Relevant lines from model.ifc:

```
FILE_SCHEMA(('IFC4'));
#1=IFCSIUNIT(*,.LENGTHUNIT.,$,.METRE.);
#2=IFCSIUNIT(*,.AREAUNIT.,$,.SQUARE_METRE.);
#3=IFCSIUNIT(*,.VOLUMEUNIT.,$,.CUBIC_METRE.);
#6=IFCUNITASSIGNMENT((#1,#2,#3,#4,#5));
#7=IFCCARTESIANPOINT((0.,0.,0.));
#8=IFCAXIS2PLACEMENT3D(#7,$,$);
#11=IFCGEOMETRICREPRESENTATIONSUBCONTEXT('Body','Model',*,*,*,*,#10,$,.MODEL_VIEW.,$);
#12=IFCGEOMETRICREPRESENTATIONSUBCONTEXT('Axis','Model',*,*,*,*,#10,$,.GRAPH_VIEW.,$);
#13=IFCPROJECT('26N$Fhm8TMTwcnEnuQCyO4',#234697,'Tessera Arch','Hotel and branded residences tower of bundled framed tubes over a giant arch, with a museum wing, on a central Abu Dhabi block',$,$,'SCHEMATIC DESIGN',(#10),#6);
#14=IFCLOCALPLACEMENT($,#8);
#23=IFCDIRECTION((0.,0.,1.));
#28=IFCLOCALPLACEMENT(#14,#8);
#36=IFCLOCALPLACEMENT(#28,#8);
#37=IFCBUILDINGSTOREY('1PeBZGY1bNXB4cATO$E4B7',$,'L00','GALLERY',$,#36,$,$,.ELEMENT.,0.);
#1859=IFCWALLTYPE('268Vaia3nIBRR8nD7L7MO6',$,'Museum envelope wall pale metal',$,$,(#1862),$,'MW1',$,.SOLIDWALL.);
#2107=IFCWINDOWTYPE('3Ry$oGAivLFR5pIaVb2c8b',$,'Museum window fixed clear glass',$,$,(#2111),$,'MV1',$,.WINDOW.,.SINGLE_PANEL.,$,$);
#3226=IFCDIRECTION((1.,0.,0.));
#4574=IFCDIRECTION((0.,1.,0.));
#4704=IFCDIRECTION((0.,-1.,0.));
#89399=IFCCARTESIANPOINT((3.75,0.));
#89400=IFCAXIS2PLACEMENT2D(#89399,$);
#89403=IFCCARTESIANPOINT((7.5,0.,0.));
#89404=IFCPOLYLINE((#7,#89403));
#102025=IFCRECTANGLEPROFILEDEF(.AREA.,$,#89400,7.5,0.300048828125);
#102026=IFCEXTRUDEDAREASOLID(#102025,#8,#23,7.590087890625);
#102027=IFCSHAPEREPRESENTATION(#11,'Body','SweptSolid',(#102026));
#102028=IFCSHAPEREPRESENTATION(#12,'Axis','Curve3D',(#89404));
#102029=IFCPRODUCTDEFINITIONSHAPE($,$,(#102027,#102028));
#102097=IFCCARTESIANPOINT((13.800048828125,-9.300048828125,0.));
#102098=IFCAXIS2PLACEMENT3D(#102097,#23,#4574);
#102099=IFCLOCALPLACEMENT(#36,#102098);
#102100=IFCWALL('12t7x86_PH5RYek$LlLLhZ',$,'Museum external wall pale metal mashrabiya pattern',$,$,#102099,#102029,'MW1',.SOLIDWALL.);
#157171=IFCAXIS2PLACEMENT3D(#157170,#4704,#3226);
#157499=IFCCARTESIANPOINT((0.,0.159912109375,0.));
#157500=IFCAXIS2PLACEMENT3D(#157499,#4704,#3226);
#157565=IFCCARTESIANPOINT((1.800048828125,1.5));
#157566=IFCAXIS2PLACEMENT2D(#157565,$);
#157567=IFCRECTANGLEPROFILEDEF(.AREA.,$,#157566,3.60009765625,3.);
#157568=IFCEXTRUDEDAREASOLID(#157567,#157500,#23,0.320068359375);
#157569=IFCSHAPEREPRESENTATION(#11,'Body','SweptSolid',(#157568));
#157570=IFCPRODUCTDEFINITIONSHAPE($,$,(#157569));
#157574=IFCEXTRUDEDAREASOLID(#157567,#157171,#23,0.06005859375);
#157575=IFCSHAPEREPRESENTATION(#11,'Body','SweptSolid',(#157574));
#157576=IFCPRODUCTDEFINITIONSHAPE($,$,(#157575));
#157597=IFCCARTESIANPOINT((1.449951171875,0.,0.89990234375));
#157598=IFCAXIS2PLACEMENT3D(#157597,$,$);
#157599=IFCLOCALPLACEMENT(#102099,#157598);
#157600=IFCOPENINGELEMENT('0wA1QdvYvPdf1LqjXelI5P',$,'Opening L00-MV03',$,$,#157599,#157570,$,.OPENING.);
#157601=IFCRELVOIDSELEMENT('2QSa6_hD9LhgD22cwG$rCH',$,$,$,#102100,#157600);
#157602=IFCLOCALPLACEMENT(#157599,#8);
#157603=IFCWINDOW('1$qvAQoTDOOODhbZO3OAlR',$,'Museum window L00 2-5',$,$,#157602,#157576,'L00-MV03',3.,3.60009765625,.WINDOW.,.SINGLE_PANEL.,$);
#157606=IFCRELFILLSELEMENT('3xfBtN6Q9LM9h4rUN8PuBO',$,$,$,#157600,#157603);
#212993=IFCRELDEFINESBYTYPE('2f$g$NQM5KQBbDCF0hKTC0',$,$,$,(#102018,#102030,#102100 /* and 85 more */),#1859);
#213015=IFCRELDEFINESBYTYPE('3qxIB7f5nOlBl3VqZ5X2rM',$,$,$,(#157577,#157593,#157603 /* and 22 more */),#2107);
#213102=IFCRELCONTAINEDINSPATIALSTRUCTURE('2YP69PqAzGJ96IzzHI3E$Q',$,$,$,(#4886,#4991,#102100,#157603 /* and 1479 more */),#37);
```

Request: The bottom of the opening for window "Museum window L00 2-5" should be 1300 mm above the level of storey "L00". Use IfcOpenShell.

```python
import numpy as np
import ifcopenshell
import ifcopenshell.api.geometry
import ifcopenshell.geom
import ifcopenshell.util.element
import ifcopenshell.util.placement
import ifcopenshell.util.shape
import ifcopenshell.util.unit

model = ifcopenshell.open("model.ifc")
unit_scale = ifcopenshell.util.unit.calculate_unit_scale(model)

window = model.by_guid("1$qvAQoTDOOODhbZO3OAlR")
opening = window.FillsVoids[0].RelatingOpeningElement
storey = ifcopenshell.util.element.get_container(window, ifc_class="IfcBuildingStorey")
level = ifcopenshell.util.placement.get_local_placement(storey.ObjectPlacement)[2, 3]

# The opening's origin need not be at the sill, so measure its lowest point.
shape = ifcopenshell.geom.create_shape(ifcopenshell.geom.settings(), opening)
bottom = ifcopenshell.util.shape.get_shape_bottom_elevation(shape, shape.geometry) / unit_scale
dz = level + 1.3 - bottom

shift = np.array([0.0, 0.0, dz])
# The window is placed relative to its opening, so it follows when the opening moves.
matrix = ifcopenshell.util.placement.get_local_placement(opening.ObjectPlacement)
matrix[:3, 3] += shift
ifcopenshell.api.geometry.edit_object_placement(
    model, product=opening, matrix=matrix, is_si=False, should_transform_children=True
)

print(f"moved by {dz * unit_scale:+.3f} m")

model.write("model_updated.ifc")
```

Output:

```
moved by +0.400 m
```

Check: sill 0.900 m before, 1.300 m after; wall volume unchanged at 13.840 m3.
